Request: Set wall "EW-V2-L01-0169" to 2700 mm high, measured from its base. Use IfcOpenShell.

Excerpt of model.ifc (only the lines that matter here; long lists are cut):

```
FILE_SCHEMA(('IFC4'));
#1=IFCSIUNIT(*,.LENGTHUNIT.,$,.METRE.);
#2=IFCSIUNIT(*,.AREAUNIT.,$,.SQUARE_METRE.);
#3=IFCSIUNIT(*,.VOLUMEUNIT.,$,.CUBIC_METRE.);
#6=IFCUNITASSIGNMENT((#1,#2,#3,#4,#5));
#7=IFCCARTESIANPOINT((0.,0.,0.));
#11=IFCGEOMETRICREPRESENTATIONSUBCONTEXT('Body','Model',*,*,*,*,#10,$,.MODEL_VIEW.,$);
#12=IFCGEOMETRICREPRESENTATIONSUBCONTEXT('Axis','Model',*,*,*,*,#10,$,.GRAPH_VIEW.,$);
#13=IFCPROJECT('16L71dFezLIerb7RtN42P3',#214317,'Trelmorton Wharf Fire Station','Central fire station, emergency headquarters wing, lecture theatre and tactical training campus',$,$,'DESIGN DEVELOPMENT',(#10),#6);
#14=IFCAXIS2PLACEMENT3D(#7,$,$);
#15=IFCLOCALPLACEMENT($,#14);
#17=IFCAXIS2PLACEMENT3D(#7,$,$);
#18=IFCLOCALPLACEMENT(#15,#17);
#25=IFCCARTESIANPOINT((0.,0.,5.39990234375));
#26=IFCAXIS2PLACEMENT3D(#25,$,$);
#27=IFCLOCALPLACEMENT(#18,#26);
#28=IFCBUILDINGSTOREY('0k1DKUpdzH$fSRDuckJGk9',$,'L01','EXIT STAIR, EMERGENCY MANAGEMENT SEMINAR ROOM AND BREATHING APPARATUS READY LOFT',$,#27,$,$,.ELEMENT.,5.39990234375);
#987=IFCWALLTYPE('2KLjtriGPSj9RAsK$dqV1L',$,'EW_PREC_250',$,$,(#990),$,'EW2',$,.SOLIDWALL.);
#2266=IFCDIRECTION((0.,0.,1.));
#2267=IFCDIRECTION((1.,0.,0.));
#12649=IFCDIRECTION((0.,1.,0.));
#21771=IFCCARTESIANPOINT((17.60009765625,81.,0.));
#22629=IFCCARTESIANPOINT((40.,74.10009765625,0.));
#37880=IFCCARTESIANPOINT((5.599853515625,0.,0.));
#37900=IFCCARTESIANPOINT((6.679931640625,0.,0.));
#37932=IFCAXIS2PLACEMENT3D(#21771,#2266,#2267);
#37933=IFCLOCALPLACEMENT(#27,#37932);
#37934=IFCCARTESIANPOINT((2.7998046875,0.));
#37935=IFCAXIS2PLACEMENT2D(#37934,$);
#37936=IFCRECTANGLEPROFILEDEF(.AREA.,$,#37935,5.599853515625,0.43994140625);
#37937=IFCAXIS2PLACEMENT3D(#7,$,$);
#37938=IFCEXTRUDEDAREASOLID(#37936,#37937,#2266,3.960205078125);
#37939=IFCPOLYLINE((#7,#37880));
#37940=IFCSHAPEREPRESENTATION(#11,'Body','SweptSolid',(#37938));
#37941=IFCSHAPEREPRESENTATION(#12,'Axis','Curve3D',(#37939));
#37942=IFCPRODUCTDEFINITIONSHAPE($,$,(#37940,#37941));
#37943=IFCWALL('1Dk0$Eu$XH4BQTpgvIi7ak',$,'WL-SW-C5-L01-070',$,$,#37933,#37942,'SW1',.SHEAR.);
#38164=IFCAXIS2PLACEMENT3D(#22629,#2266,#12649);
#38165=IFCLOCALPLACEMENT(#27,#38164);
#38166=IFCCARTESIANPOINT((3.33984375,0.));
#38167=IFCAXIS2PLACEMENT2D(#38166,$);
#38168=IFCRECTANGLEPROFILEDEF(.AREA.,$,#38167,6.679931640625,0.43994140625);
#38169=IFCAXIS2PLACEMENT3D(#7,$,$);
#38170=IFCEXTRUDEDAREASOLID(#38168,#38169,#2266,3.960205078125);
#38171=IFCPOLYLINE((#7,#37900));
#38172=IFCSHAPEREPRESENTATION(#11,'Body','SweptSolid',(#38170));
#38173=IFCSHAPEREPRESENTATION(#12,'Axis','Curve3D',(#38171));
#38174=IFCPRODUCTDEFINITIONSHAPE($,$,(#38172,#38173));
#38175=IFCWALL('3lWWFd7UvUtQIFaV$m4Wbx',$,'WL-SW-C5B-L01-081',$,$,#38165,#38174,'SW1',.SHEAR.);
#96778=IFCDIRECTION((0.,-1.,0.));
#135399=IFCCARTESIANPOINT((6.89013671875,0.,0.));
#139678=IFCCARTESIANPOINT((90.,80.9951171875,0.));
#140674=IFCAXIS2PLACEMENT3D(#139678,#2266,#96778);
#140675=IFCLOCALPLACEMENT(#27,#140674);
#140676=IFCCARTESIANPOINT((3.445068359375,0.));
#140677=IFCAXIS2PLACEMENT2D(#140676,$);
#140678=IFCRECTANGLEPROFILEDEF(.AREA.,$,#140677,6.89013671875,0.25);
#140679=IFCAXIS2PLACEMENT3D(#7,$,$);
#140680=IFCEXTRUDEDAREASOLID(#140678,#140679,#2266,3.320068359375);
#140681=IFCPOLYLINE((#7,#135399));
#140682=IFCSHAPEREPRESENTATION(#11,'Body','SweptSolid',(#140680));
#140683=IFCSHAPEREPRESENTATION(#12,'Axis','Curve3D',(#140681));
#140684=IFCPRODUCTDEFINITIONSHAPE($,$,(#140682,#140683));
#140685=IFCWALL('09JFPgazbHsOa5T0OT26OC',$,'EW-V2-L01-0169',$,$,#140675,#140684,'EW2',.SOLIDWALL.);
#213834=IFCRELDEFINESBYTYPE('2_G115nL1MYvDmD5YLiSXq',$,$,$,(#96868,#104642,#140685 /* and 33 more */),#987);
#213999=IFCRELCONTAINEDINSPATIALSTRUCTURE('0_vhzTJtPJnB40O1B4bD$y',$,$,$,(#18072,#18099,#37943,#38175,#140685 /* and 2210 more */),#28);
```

```python
import ifcopenshell
import ifcopenshell.geom
import ifcopenshell.util.representation
import ifcopenshell.util.shape

model = ifcopenshell.open("model.ifc")
settings = ifcopenshell.geom.settings()


def volume(element):
    """Net volume in cubic metres, openings subtracted."""
    shape = ifcopenshell.geom.create_shape(settings, element)
    return ifcopenshell.util.shape.get_volume(shape.geometry)


wall = model.by_id(140685)
before = volume(wall)

body = ifcopenshell.util.representation.get_representation(wall, "Model", "Body")
solid = body.Items[0]
old_height = solid.Depth
solid.Depth = 2.7
after = volume(wall)

print(f"height {old_height:g} -> {solid.Depth:g}, volume {before:.3f} -> {after:.3f} m3")

model.write("model_v2.ifc")
```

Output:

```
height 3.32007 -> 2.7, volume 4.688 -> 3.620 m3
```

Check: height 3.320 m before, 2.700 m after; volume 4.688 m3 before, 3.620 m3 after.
